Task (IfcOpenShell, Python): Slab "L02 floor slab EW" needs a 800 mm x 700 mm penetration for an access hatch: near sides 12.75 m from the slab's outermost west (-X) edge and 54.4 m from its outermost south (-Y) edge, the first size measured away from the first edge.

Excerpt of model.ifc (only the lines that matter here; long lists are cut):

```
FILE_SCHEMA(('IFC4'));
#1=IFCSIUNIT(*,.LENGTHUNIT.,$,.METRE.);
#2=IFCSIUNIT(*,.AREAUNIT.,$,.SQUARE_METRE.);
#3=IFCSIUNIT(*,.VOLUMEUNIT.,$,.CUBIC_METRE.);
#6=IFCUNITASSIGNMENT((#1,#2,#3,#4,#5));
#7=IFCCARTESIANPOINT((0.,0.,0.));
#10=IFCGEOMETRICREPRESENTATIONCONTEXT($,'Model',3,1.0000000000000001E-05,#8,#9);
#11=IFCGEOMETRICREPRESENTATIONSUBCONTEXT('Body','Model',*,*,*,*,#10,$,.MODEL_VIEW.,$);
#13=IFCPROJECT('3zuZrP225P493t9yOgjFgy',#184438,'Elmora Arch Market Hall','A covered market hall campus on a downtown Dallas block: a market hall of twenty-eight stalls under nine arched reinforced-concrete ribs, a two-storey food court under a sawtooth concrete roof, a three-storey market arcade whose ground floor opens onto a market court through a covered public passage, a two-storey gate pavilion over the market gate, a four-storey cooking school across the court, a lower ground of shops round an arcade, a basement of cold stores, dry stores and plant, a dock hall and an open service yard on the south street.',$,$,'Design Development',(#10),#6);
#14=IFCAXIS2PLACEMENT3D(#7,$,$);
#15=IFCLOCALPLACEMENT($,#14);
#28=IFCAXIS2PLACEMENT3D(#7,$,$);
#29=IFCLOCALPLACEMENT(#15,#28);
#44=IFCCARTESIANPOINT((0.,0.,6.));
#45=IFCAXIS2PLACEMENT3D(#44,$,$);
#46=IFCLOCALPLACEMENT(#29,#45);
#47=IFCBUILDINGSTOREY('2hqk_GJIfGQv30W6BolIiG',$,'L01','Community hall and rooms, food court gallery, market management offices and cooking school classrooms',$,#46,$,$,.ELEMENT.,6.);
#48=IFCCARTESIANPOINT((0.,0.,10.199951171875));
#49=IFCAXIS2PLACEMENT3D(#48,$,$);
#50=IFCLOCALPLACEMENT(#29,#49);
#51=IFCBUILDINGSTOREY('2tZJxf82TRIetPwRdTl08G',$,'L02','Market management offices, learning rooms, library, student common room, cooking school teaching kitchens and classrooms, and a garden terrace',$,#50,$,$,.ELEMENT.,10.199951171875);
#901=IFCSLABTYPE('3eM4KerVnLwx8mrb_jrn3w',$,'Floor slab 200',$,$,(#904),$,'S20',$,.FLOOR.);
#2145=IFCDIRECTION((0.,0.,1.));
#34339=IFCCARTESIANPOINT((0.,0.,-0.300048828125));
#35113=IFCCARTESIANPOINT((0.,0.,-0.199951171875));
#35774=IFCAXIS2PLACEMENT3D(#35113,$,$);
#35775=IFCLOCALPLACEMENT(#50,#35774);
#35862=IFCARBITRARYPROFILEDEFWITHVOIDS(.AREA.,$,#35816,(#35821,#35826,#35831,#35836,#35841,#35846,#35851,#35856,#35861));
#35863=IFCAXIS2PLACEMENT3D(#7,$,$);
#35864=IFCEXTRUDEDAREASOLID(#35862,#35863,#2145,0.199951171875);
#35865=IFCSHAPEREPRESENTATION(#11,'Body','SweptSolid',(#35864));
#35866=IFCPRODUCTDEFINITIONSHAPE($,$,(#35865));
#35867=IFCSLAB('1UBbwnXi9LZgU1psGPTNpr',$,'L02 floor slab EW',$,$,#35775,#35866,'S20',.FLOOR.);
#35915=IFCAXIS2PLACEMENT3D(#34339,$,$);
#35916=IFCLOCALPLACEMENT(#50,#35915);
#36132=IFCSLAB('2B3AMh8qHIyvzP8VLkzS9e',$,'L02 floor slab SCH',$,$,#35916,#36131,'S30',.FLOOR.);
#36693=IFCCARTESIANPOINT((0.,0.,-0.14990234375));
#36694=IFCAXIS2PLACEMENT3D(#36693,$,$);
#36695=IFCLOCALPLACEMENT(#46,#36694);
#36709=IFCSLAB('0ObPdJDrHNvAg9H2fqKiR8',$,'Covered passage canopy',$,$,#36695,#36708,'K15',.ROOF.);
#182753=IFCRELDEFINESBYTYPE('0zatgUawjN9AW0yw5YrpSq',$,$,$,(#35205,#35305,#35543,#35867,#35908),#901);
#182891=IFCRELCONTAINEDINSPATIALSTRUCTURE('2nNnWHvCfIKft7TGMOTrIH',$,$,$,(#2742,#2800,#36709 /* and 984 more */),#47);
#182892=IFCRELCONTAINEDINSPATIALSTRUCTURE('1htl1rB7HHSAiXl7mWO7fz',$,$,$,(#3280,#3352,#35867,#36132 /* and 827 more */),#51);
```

```python
import numpy as np
import ifcopenshell
import ifcopenshell.api.feature
import ifcopenshell.api.geometry
import ifcopenshell.api.root
import ifcopenshell.geom
import ifcopenshell.util.placement
import ifcopenshell.util.representation
import ifcopenshell.util.shape
import ifcopenshell.util.unit

model = ifcopenshell.open("model.ifc")
unit_scale = ifcopenshell.util.unit.calculate_unit_scale(model)
settings = ifcopenshell.geom.settings()


def volume(element):
    """Net volume in cubic metres, openings subtracted."""
    shape = ifcopenshell.geom.create_shape(settings, element)
    return ifcopenshell.util.shape.get_volume(shape.geometry)


slab = model.by_guid("1UBbwnXi9LZgU1psGPTNpr")
before = volume(slab)

# Extent in the slab's own axes, in metres. The edges named are its -X and -Y sides.
slab_shape = ifcopenshell.geom.create_shape(settings, slab)
vertices = ifcopenshell.util.shape.get_vertices(slab_shape.geometry)
x_min, y_min, bottom = vertices.min(axis=0)
top = vertices[:, 2].max()

opening = ifcopenshell.api.root.create_entity(model, ifc_class="IfcOpeningElement", name="Access hatch opening", predefined_type="OPENING")
context = ifcopenshell.util.representation.get_context(model, "Model", "Body", "MODEL_VIEW")
width, depth = 0.8, 0.7
outline = [(0.0, 0.0), (width, 0.0), (width, depth), (0.0, depth), (0.0, 0.0)]
# Overshoot both faces by 50 mm so the cut is clean.
shape = ifcopenshell.api.geometry.add_slab_representation(
    model, context=context, depth=top - bottom + 0.1, polyline=outline
)
ifcopenshell.api.geometry.assign_representation(model, product=opening, representation=shape)

matrix = ifcopenshell.util.placement.get_local_placement(slab.ObjectPlacement)
matrix[:, 3] = matrix @ np.append(np.array([x_min + 12.75, y_min + 54.4, bottom - 0.05]) / unit_scale, 1.0)
ifcopenshell.api.geometry.edit_object_placement(model, product=opening, matrix=matrix, is_si=False)
ifcopenshell.api.feature.add_feature(model, feature=opening, element=slab)

after = volume(slab)

print(f"slab volume {before:.3f} -> {after:.3f} m3")

model.write("model_updated.ifc")
```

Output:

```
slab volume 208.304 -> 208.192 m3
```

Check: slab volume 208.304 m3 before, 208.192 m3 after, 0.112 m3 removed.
